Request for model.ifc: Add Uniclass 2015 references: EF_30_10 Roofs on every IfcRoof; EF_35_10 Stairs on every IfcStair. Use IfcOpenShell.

First a look at what the model holds.

```python
import ifcopenshell

model = ifcopenshell.open("model.ifc")
print(model.schema)
print("classifications:", [c.Name for c in model.by_type("IfcClassification")])
for ifc_class in ("IfcDoor", "IfcRoof", "IfcStair", "IfcWall", "IfcWindow"):
    print(ifc_class, len(model.by_type(ifc_class)))
```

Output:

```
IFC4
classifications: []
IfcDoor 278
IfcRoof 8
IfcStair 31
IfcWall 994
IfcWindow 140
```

```python
import ifcopenshell
import ifcopenshell.api.classification

model = ifcopenshell.open("model.ifc")

system = ifcopenshell.api.classification.add_classification(model, classification="Uniclass 2015")

codes = {
    "IfcRoof": ("EF_30_10", "Roofs"),
    "IfcStair": ("EF_35_10", "Stairs"),
}
for ifc_class, (code, name) in codes.items():
    products = model.by_type(ifc_class)
    ifcopenshell.api.classification.add_reference(
        model, products=products, classification=system, identification=code, name=name
    )
    print(code, len(products))

model.write("model_edited.ifc")
```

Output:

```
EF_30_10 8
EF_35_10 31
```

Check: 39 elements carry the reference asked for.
